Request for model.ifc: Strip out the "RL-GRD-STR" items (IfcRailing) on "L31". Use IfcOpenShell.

First a look at what the model holds.

```python
import ifcopenshell
import ifcopenshell.util.element

model = ifcopenshell.open("model.ifc")
print(model.schema)
storey = next(s for s in model.by_type("IfcBuildingStorey") if s.Name == "L31")
railings = [e for e in ifcopenshell.util.element.get_decomposition(storey) if e.is_a("IfcRailing")]
seen = {}
for e in railings:
    element_type = ifcopenshell.util.element.get_type(e)
    name = element_type.Name if element_type not in (None, e) else None
    seen[name] = seen.get(name, 0) + 1
for name, count in sorted(seen.items(), key=str):
    print(count, "x", name)
```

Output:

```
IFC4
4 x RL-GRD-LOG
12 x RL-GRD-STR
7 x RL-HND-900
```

```python
import ifcopenshell
import ifcopenshell.api.root
import ifcopenshell.util.element

model = ifcopenshell.open("model.ifc")

storey = next(s for s in model.by_type("IfcBuildingStorey") if s.Name == "L31")
railings = [e for e in ifcopenshell.util.element.get_decomposition(storey) if e.is_a("IfcRailing")]
targets = [e for e in railings if (t := ifcopenshell.util.element.get_type(e)) not in (None, e) and t.Name == "RL-GRD-STR"]

for e in targets:
    ifcopenshell.api.root.remove_product(model, product=e)
print(len(targets), "removed")

model.write("model_edited.ifc")
```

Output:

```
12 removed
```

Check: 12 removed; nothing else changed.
